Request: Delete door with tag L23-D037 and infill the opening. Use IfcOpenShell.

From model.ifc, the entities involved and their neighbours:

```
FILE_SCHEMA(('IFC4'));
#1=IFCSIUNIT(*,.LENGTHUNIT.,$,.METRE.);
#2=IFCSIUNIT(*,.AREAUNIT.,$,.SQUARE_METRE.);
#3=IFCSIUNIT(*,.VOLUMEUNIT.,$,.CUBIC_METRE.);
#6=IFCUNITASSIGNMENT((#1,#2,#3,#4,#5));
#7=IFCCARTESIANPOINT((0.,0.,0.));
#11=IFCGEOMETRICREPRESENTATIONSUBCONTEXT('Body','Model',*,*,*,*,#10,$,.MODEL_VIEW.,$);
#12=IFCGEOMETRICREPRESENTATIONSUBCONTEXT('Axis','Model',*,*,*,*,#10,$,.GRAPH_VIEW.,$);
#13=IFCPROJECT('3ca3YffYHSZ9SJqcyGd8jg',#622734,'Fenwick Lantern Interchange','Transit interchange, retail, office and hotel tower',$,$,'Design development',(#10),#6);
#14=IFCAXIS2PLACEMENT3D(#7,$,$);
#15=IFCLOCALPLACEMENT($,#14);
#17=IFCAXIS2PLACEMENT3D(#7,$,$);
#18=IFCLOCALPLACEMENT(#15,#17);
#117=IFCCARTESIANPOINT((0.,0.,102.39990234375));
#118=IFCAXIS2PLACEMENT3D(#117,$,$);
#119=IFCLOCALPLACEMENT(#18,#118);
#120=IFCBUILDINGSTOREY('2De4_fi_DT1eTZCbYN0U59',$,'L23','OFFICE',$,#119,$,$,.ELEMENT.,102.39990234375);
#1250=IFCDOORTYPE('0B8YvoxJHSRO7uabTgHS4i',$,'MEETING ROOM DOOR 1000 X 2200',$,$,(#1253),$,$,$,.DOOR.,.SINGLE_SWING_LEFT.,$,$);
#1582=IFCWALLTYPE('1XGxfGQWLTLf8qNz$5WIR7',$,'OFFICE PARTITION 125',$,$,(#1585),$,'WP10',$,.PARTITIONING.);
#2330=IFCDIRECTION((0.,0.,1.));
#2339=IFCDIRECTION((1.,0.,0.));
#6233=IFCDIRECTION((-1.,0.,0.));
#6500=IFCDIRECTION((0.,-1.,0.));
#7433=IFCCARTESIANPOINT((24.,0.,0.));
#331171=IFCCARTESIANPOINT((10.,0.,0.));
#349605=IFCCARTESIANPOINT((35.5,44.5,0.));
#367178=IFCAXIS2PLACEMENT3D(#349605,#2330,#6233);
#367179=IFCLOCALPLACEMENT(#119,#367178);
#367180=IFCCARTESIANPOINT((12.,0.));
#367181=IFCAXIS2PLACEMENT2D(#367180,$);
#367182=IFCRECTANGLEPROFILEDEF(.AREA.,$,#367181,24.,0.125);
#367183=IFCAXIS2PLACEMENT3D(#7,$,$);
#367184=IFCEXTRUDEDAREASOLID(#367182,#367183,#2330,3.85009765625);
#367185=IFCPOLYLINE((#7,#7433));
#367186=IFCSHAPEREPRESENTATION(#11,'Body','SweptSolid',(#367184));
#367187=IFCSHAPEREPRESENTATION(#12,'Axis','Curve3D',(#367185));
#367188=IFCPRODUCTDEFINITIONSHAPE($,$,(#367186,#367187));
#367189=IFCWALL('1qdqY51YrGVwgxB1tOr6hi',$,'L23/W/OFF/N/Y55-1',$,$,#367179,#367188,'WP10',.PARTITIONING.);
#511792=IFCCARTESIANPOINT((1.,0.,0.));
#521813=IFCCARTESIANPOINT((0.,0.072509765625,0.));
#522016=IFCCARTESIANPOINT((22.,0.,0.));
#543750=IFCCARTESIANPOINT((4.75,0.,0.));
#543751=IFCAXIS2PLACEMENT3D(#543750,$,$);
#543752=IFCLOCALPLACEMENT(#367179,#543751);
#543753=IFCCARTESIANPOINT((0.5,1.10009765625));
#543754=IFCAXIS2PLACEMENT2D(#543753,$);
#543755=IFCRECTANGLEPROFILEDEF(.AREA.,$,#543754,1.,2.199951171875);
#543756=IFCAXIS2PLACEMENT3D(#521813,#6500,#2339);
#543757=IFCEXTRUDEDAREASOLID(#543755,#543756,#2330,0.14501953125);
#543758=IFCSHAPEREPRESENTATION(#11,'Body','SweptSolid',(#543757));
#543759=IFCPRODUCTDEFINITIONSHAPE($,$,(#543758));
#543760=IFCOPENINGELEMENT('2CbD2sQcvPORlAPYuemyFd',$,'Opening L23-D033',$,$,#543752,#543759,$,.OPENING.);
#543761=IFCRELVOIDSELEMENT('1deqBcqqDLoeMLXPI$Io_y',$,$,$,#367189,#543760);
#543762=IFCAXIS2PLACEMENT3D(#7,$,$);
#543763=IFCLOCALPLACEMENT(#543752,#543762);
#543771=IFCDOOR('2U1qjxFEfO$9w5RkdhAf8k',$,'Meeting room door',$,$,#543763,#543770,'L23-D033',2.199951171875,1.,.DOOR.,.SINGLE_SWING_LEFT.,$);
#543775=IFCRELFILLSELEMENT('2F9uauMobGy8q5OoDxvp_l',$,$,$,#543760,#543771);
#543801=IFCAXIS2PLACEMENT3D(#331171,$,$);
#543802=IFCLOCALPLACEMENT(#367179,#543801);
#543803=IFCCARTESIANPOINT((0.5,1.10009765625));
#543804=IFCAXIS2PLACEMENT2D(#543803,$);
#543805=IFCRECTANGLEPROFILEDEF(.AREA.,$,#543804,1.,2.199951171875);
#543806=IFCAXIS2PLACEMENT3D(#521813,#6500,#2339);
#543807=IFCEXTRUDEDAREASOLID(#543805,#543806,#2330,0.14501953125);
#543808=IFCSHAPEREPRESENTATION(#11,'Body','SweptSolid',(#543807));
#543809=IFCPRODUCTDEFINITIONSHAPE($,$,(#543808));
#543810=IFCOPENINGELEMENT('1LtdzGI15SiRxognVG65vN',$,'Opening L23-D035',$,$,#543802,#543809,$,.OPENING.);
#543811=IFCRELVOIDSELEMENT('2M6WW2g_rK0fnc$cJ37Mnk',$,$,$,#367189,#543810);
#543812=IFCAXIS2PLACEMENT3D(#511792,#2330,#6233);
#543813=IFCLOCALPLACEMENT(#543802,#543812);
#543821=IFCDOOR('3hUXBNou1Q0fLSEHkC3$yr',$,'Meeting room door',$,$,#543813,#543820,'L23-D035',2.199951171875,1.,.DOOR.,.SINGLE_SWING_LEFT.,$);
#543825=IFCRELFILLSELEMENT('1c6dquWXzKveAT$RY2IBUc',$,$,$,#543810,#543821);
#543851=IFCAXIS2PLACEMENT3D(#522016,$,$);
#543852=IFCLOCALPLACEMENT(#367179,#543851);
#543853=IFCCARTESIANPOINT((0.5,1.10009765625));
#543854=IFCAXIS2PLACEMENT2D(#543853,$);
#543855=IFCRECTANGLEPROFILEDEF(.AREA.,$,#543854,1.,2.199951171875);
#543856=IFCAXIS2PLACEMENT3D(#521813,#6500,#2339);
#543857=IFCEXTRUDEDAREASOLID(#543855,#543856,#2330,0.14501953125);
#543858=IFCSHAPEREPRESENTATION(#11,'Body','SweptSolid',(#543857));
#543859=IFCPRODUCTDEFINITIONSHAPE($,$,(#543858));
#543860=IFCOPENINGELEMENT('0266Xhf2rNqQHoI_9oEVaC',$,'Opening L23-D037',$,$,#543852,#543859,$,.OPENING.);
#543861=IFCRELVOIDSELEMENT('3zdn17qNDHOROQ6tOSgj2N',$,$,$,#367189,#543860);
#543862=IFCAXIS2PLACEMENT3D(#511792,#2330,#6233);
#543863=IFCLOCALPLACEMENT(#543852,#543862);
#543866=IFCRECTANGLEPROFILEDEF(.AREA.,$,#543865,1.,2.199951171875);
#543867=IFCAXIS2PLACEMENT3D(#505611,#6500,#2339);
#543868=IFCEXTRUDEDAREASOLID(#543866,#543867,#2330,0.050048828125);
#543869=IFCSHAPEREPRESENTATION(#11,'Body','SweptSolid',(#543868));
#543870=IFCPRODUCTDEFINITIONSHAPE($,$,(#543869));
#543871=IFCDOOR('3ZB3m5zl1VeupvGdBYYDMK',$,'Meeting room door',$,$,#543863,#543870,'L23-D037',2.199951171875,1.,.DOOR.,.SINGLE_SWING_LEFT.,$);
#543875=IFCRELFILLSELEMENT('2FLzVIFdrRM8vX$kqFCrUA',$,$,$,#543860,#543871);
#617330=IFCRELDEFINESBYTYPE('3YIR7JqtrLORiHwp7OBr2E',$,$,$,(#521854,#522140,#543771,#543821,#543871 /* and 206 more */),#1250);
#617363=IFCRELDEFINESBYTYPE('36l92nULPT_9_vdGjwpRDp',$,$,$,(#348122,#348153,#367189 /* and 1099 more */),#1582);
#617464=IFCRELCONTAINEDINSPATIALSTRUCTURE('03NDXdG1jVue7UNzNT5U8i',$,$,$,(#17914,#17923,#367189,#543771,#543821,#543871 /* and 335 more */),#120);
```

```python
import ifcopenshell
import ifcopenshell.api.feature
import ifcopenshell.api.root
import ifcopenshell.geom
import ifcopenshell.util.shape

model = ifcopenshell.open("model.ifc")
settings = ifcopenshell.geom.settings()


def volume(element):
    """Net volume in cubic metres, openings subtracted."""
    shape = ifcopenshell.geom.create_shape(settings, element)
    return ifcopenshell.util.shape.get_volume(shape.geometry)


door = model.by_guid("3ZB3m5zl1VeupvGdBYYDMK")
opening = door.FillsVoids[0].RelatingOpeningElement
wall = opening.VoidsElements[0].RelatingBuildingElement
before = volume(wall)

ifcopenshell.api.root.remove_product(model, product=door)
ifcopenshell.api.feature.remove_feature(model, feature=opening)

after = volume(wall)

print(f"wall volume {before:.3f} -> {after:.3f} m3")

model.write("model-out.ifc")
```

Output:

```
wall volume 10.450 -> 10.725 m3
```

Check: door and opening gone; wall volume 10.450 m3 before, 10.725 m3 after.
